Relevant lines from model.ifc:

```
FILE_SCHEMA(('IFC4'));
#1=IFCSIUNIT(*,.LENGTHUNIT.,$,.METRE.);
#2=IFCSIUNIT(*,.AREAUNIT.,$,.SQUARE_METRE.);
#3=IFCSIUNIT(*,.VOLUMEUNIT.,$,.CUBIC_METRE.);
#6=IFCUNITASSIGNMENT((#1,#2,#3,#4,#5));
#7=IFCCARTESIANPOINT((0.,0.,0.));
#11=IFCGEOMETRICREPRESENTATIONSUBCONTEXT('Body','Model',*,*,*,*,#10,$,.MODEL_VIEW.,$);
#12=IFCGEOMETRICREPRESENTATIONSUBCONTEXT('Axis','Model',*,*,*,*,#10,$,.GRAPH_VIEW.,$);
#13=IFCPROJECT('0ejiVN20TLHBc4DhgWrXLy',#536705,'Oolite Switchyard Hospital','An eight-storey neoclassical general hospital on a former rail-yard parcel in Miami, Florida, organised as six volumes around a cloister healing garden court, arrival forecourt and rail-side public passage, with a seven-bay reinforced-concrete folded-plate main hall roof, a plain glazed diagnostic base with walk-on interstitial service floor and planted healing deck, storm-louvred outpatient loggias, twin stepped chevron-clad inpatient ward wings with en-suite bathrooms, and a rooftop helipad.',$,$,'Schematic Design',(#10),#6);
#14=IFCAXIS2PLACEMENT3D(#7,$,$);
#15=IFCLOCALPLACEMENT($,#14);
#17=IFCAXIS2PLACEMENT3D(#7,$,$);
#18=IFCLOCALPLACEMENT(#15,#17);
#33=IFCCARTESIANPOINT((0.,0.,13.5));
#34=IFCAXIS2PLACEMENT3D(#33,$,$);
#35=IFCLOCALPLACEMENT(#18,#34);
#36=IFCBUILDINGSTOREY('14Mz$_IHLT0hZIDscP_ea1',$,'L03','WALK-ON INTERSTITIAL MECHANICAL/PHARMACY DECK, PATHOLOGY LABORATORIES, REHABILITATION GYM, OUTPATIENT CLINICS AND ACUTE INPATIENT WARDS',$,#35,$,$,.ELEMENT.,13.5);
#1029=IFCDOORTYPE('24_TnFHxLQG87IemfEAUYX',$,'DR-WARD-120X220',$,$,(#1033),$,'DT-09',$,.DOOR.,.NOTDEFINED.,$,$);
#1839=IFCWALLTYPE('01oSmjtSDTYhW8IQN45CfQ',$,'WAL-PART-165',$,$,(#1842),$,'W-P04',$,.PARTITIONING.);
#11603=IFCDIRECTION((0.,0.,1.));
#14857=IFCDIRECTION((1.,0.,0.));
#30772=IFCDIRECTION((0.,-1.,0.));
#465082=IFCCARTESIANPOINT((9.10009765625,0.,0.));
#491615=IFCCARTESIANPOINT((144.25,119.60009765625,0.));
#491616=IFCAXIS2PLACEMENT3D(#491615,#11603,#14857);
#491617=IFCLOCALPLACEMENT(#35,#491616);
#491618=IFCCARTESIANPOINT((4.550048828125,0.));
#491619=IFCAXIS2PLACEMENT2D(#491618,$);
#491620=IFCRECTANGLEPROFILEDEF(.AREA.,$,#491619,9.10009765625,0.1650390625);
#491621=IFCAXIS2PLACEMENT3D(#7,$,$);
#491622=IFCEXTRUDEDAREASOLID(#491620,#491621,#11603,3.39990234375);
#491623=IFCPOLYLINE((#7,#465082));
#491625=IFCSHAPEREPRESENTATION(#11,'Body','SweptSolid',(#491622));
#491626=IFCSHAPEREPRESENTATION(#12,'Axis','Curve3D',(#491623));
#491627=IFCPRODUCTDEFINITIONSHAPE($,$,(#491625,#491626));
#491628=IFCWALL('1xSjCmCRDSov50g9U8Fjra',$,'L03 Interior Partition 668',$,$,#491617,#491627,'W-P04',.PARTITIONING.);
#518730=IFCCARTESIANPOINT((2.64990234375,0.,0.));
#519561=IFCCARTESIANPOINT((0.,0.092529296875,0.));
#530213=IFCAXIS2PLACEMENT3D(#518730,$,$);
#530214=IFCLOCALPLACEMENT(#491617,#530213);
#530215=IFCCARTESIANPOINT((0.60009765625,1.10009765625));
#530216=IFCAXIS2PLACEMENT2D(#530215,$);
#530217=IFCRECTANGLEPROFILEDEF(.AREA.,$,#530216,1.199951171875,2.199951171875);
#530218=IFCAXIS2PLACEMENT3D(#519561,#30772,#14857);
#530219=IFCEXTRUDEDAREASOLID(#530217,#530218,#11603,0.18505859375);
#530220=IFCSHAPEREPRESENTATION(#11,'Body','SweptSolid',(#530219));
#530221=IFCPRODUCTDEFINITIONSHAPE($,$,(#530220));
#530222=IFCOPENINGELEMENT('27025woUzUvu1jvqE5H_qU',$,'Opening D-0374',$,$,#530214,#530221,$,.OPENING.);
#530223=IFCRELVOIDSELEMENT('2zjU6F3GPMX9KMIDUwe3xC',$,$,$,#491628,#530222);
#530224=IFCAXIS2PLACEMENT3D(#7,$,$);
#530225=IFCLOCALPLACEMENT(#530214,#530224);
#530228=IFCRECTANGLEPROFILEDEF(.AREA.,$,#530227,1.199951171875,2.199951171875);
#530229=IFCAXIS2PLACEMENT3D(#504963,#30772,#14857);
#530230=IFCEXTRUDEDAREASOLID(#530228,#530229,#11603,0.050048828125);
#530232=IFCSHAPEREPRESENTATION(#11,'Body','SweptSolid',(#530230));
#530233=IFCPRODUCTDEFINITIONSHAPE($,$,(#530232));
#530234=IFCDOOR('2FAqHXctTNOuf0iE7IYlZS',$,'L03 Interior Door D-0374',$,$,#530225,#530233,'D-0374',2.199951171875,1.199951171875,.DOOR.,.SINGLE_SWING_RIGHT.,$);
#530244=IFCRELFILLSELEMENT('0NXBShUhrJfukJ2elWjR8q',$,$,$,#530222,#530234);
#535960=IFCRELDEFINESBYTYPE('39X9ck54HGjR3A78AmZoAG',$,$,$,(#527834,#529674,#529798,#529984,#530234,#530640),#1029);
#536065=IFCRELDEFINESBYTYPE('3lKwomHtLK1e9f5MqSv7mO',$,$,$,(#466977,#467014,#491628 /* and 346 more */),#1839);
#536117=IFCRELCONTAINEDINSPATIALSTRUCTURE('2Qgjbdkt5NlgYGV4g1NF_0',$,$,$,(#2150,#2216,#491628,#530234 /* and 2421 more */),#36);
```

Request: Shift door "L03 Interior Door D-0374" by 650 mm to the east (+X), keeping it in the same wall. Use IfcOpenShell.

```python
import ifcopenshell
import ifcopenshell.api.geometry
import ifcopenshell.util.placement
import ifcopenshell.util.unit

model = ifcopenshell.open("model.ifc")
unit_scale = ifcopenshell.util.unit.calculate_unit_scale(model)

door = model.by_guid("2FAqHXctTNOuf0iE7IYlZS")
opening = door.FillsVoids[0].RelatingOpeningElement
wall = opening.VoidsElements[0].RelatingBuildingElement

wall_matrix = ifcopenshell.util.placement.get_local_placement(wall.ObjectPlacement)
shift = wall_matrix[:3, 0] * 0.65 / unit_scale
before = ifcopenshell.util.placement.get_local_placement(door.ObjectPlacement)[:3, 3].copy()

# The door is placed relative to its opening, so it follows when the opening moves.
matrix = ifcopenshell.util.placement.get_local_placement(opening.ObjectPlacement)
matrix[:3, 3] += shift
ifcopenshell.api.geometry.edit_object_placement(
    model, product=opening, matrix=matrix, is_si=False, should_transform_children=True
)

after = ifcopenshell.util.placement.get_local_placement(door.ObjectPlacement)[:3, 3]
print("door moved by", (after - before).round(3) + 0.0)

model.write("model_rev.ifc")
```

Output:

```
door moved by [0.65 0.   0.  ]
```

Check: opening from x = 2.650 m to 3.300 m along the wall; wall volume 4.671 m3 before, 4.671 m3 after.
